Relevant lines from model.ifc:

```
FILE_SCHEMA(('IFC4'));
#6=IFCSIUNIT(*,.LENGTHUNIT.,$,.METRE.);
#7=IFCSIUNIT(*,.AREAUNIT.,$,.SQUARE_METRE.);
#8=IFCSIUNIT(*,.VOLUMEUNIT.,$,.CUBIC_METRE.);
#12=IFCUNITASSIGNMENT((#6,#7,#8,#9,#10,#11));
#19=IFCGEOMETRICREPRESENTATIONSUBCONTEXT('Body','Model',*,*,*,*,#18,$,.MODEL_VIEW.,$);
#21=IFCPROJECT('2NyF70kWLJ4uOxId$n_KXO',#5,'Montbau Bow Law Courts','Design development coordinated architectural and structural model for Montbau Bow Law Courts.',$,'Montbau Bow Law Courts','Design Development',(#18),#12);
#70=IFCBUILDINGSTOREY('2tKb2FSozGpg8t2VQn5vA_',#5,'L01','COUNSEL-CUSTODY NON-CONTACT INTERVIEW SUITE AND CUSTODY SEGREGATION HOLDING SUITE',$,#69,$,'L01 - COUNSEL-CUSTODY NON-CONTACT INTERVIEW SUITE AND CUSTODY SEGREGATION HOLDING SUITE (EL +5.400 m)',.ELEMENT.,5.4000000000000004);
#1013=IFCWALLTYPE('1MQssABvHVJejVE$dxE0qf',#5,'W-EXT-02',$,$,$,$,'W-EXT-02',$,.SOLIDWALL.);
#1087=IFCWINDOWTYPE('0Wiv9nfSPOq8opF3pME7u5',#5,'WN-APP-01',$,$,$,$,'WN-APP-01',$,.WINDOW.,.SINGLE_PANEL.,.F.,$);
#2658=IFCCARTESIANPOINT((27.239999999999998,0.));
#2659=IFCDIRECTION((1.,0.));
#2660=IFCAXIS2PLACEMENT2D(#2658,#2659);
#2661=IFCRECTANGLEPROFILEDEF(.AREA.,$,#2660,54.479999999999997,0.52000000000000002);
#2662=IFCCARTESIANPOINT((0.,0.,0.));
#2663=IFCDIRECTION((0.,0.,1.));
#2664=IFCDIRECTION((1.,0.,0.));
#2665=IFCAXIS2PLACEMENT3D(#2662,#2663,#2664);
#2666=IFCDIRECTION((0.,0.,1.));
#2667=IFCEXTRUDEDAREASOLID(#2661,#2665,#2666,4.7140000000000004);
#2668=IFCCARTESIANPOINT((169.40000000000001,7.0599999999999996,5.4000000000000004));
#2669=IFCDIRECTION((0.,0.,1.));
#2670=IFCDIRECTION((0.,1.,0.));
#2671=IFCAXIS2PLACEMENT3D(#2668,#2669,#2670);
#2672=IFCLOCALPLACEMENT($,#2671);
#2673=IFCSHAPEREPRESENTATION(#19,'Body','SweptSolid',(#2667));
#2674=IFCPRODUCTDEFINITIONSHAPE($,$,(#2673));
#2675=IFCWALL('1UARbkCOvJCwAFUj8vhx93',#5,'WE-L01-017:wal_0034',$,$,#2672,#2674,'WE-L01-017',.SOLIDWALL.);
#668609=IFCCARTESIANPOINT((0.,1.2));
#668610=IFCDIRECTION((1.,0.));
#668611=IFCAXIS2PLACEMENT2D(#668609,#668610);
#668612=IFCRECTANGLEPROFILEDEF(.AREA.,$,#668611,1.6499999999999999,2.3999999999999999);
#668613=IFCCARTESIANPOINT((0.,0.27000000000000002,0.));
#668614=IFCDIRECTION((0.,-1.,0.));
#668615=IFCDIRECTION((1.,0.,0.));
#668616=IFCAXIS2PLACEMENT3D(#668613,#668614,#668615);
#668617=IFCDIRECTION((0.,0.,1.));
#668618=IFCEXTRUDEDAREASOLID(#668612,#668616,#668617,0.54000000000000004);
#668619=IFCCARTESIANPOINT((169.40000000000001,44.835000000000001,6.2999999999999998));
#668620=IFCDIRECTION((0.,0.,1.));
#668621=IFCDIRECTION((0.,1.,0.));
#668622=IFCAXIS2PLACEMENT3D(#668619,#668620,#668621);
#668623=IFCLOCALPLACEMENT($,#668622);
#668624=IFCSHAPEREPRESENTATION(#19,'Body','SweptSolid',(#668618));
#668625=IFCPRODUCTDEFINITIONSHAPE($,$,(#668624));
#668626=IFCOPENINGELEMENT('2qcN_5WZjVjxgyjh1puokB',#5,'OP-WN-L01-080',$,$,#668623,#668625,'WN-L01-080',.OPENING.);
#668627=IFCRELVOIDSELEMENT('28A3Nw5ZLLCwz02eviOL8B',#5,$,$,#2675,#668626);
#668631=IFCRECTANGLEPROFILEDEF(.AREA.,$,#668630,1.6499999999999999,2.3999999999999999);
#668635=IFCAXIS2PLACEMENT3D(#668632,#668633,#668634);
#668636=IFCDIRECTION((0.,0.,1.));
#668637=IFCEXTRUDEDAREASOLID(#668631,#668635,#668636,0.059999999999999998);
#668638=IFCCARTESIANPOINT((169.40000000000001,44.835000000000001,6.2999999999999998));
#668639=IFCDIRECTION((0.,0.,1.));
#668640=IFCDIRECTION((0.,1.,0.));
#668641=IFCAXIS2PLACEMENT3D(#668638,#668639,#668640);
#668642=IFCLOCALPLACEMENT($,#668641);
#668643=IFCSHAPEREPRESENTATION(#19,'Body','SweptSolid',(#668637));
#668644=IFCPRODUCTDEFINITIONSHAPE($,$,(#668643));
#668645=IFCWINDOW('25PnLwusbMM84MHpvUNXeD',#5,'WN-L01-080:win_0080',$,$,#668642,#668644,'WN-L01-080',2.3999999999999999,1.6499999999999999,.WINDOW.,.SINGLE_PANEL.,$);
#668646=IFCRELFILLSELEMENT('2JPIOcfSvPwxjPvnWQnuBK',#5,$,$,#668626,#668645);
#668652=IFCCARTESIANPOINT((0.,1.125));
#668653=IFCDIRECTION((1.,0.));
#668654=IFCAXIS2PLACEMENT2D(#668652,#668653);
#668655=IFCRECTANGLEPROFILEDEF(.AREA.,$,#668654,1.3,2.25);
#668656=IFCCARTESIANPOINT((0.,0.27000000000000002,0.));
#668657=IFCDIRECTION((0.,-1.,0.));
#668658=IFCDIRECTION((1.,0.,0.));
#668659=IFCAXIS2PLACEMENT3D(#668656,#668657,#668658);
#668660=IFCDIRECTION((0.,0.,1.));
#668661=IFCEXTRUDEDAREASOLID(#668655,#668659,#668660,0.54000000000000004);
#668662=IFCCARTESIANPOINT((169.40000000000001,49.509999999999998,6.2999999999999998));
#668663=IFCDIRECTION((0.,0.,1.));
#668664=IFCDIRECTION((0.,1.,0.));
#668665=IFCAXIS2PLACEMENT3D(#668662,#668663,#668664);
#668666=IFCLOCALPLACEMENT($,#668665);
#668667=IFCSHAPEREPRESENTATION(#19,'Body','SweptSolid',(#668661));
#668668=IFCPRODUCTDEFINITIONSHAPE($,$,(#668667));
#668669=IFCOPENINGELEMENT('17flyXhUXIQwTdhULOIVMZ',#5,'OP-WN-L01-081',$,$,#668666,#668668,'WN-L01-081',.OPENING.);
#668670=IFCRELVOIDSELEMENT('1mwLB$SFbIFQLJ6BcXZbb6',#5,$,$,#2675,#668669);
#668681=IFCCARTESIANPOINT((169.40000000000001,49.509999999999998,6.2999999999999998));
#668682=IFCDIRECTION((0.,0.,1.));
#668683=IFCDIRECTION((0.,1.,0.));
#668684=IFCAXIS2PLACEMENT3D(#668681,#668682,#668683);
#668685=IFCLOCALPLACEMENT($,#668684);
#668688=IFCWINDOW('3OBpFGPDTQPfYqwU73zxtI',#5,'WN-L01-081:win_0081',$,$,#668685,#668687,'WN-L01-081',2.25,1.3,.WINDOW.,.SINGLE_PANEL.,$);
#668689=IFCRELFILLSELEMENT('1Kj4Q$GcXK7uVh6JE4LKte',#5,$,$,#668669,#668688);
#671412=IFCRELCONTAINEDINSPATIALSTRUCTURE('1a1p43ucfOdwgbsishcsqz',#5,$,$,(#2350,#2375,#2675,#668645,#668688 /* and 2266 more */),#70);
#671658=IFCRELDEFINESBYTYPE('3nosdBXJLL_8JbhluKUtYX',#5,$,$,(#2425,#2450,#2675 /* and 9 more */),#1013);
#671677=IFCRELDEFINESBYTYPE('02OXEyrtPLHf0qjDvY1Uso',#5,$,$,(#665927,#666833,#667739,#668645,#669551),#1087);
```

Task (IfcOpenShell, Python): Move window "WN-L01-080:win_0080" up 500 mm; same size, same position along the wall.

```python
import numpy as np
import ifcopenshell
import ifcopenshell.api.geometry
import ifcopenshell.util.placement
import ifcopenshell.util.unit

model = ifcopenshell.open("model.ifc")
unit_scale = ifcopenshell.util.unit.calculate_unit_scale(model)

window = model.by_guid("25PnLwusbMM84MHpvUNXeD")
opening = window.FillsVoids[0].RelatingOpeningElement
dz = 0.5

shift = np.array([0.0, 0.0, dz])
# The window is not placed relative to its opening, so move both.
for product in (opening, window):
    matrix = ifcopenshell.util.placement.get_local_placement(product.ObjectPlacement)
    matrix[:3, 3] += shift
    ifcopenshell.api.geometry.edit_object_placement(model, product=product, matrix=matrix, is_si=False)

print(f"moved by {dz * unit_scale:+.3f} m")

model.write("model_v2.ifc")
```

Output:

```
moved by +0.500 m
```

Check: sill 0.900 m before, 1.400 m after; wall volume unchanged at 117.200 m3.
